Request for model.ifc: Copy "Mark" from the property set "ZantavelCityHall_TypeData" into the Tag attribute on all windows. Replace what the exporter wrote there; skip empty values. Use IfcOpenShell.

First a look at what the model holds.

```python
import ifcopenshell
import ifcopenshell.util.element

model = ifcopenshell.open("model.ifc")
print(model.schema)
windows = model.by_type("IfcWindow")
print(len(windows), "windows")
for e in windows[:8]:
    source = ifcopenshell.util.element.get_pset(e, "ZantavelCityHall_TypeData", "Mark")
    target = e.Tag
    print(e.id(), repr(source), repr(target), sep=" | ")
```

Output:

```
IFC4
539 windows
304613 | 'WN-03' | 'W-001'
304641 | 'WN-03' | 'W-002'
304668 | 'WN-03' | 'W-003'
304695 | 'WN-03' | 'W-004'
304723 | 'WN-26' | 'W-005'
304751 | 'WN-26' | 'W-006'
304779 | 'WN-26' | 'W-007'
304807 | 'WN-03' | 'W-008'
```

```python
import ifcopenshell
import ifcopenshell.util.element

model = ifcopenshell.open("model.ifc")

count = 0
for e in model.by_type("IfcWindow"):
    value = ifcopenshell.util.element.get_pset(e, "ZantavelCityHall_TypeData", "Mark")
    current = e.Tag
    if not value or not value.strip() or current == value:
        continue
    e.Tag = value
    count += 1

print(count, "windows updated")

model.write("model_v2.ifc")
```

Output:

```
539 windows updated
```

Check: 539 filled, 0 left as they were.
